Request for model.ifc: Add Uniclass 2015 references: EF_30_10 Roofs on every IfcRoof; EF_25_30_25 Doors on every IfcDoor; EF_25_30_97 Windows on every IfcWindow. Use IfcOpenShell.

First a look at what the model holds.

```python
import ifcopenshell

model = ifcopenshell.open("model.ifc")
print(model.schema)
print("classifications:", [c.Name for c in model.by_type("IfcClassification")])
for ifc_class in ("IfcDoor", "IfcRoof", "IfcStair", "IfcWall", "IfcWindow"):
    print(ifc_class, len(model.by_type(ifc_class)))
```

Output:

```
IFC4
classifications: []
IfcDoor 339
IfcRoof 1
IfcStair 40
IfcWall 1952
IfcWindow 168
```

```python
import ifcopenshell
import ifcopenshell.api.classification

model = ifcopenshell.open("model.ifc")

system = ifcopenshell.api.classification.add_classification(model, classification="Uniclass 2015")

codes = {
    "IfcRoof": ("EF_30_10", "Roofs"),
    "IfcDoor": ("EF_25_30_25", "Doors"),
    "IfcWindow": ("EF_25_30_97", "Windows"),
}
for ifc_class, (code, name) in codes.items():
    products = model.by_type(ifc_class)
    ifcopenshell.api.classification.add_reference(
        model, products=products, classification=system, identification=code, name=name
    )
    print(code, len(products))

model.write("model_updated.ifc")
```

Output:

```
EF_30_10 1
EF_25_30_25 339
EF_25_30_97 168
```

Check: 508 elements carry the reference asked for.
